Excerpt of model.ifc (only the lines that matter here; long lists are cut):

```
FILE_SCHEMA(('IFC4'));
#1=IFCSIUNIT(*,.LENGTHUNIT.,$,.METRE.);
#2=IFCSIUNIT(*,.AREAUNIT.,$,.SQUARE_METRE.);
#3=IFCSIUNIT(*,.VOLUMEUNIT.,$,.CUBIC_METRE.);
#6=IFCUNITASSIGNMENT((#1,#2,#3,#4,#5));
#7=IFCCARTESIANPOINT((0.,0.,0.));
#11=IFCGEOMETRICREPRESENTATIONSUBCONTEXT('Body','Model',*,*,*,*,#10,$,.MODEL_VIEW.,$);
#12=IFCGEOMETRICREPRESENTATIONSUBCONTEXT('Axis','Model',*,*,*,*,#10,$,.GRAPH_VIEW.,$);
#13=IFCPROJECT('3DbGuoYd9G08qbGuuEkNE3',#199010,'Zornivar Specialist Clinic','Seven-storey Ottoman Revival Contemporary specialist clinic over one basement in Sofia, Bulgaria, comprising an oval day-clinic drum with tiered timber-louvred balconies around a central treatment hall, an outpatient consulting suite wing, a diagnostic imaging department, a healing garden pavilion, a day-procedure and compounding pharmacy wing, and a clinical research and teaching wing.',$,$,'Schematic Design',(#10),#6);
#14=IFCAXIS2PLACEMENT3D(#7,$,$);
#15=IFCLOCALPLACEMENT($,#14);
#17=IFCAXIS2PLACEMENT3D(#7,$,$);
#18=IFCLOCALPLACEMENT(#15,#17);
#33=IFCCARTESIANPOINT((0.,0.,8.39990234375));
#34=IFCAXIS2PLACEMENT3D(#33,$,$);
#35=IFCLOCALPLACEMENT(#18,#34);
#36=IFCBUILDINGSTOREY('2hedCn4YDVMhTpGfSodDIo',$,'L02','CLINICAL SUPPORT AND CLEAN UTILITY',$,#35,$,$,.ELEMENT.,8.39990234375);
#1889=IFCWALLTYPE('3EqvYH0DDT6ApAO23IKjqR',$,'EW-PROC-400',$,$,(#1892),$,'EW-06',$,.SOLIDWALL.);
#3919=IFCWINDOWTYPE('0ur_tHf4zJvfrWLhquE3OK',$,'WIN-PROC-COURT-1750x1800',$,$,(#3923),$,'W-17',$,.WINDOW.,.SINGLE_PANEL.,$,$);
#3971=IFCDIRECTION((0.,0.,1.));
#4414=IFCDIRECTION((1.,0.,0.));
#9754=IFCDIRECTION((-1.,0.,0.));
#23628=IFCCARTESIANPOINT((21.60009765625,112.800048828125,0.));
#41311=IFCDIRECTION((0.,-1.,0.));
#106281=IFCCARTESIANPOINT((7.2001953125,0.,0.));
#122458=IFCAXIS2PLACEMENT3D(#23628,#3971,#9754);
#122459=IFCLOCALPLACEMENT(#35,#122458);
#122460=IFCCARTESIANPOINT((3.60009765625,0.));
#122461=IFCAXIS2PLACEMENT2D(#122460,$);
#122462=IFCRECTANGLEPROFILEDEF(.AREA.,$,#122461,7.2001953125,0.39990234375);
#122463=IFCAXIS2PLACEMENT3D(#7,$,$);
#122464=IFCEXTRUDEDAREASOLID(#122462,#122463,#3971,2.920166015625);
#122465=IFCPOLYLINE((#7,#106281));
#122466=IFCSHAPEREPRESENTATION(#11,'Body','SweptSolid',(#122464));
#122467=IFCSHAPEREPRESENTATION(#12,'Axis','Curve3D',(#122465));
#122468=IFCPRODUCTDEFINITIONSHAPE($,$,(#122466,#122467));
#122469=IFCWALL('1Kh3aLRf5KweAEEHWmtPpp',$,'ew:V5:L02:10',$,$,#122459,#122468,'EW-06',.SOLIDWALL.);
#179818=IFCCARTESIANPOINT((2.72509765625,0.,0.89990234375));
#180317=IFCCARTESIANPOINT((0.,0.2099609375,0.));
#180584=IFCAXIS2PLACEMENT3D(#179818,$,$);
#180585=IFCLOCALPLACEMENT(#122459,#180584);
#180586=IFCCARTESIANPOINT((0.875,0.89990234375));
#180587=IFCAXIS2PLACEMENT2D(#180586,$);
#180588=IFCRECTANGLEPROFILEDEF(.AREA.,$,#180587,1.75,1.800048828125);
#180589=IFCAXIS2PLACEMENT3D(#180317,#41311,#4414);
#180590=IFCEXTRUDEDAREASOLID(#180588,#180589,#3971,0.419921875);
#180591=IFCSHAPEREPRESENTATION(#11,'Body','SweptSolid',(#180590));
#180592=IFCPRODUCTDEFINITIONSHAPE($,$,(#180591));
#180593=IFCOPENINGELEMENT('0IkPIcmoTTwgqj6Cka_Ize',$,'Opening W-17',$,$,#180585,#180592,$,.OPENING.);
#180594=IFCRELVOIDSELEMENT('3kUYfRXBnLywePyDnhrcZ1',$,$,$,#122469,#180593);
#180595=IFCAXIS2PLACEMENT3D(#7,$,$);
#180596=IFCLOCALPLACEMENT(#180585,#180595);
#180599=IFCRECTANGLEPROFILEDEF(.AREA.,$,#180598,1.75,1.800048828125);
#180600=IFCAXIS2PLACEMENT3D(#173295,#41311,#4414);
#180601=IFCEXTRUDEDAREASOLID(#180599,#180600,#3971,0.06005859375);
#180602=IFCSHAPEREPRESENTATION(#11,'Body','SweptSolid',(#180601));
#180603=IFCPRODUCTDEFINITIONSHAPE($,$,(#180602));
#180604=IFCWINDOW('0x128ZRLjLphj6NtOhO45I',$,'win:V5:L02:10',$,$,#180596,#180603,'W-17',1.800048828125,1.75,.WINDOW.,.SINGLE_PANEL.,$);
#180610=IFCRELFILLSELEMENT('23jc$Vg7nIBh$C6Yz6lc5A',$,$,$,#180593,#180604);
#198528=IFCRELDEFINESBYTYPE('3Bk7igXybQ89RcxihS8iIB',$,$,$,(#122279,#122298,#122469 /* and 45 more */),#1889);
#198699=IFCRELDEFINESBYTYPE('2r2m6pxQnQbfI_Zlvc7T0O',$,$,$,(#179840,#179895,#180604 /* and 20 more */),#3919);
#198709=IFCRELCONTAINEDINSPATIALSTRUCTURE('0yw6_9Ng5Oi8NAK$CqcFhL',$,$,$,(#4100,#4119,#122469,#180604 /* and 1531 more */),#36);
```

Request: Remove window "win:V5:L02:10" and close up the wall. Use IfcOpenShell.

```python
import ifcopenshell
import ifcopenshell.api.feature
import ifcopenshell.api.root
import ifcopenshell.geom
import ifcopenshell.util.shape

model = ifcopenshell.open("model.ifc")
settings = ifcopenshell.geom.settings()


def volume(element):
    """Net volume in cubic metres, openings subtracted."""
    shape = ifcopenshell.geom.create_shape(settings, element)
    return ifcopenshell.util.shape.get_volume(shape.geometry)


window = model.by_guid("0x128ZRLjLphj6NtOhO45I")
opening = window.FillsVoids[0].RelatingOpeningElement
wall = opening.VoidsElements[0].RelatingBuildingElement
before = volume(wall)

ifcopenshell.api.root.remove_product(model, product=window)
ifcopenshell.api.feature.remove_feature(model, feature=opening)

after = volume(wall)

print(f"wall volume {before:.3f} -> {after:.3f} m3")

model.write("model-out.ifc")
```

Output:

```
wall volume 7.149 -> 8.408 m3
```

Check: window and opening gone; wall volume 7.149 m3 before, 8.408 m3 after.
